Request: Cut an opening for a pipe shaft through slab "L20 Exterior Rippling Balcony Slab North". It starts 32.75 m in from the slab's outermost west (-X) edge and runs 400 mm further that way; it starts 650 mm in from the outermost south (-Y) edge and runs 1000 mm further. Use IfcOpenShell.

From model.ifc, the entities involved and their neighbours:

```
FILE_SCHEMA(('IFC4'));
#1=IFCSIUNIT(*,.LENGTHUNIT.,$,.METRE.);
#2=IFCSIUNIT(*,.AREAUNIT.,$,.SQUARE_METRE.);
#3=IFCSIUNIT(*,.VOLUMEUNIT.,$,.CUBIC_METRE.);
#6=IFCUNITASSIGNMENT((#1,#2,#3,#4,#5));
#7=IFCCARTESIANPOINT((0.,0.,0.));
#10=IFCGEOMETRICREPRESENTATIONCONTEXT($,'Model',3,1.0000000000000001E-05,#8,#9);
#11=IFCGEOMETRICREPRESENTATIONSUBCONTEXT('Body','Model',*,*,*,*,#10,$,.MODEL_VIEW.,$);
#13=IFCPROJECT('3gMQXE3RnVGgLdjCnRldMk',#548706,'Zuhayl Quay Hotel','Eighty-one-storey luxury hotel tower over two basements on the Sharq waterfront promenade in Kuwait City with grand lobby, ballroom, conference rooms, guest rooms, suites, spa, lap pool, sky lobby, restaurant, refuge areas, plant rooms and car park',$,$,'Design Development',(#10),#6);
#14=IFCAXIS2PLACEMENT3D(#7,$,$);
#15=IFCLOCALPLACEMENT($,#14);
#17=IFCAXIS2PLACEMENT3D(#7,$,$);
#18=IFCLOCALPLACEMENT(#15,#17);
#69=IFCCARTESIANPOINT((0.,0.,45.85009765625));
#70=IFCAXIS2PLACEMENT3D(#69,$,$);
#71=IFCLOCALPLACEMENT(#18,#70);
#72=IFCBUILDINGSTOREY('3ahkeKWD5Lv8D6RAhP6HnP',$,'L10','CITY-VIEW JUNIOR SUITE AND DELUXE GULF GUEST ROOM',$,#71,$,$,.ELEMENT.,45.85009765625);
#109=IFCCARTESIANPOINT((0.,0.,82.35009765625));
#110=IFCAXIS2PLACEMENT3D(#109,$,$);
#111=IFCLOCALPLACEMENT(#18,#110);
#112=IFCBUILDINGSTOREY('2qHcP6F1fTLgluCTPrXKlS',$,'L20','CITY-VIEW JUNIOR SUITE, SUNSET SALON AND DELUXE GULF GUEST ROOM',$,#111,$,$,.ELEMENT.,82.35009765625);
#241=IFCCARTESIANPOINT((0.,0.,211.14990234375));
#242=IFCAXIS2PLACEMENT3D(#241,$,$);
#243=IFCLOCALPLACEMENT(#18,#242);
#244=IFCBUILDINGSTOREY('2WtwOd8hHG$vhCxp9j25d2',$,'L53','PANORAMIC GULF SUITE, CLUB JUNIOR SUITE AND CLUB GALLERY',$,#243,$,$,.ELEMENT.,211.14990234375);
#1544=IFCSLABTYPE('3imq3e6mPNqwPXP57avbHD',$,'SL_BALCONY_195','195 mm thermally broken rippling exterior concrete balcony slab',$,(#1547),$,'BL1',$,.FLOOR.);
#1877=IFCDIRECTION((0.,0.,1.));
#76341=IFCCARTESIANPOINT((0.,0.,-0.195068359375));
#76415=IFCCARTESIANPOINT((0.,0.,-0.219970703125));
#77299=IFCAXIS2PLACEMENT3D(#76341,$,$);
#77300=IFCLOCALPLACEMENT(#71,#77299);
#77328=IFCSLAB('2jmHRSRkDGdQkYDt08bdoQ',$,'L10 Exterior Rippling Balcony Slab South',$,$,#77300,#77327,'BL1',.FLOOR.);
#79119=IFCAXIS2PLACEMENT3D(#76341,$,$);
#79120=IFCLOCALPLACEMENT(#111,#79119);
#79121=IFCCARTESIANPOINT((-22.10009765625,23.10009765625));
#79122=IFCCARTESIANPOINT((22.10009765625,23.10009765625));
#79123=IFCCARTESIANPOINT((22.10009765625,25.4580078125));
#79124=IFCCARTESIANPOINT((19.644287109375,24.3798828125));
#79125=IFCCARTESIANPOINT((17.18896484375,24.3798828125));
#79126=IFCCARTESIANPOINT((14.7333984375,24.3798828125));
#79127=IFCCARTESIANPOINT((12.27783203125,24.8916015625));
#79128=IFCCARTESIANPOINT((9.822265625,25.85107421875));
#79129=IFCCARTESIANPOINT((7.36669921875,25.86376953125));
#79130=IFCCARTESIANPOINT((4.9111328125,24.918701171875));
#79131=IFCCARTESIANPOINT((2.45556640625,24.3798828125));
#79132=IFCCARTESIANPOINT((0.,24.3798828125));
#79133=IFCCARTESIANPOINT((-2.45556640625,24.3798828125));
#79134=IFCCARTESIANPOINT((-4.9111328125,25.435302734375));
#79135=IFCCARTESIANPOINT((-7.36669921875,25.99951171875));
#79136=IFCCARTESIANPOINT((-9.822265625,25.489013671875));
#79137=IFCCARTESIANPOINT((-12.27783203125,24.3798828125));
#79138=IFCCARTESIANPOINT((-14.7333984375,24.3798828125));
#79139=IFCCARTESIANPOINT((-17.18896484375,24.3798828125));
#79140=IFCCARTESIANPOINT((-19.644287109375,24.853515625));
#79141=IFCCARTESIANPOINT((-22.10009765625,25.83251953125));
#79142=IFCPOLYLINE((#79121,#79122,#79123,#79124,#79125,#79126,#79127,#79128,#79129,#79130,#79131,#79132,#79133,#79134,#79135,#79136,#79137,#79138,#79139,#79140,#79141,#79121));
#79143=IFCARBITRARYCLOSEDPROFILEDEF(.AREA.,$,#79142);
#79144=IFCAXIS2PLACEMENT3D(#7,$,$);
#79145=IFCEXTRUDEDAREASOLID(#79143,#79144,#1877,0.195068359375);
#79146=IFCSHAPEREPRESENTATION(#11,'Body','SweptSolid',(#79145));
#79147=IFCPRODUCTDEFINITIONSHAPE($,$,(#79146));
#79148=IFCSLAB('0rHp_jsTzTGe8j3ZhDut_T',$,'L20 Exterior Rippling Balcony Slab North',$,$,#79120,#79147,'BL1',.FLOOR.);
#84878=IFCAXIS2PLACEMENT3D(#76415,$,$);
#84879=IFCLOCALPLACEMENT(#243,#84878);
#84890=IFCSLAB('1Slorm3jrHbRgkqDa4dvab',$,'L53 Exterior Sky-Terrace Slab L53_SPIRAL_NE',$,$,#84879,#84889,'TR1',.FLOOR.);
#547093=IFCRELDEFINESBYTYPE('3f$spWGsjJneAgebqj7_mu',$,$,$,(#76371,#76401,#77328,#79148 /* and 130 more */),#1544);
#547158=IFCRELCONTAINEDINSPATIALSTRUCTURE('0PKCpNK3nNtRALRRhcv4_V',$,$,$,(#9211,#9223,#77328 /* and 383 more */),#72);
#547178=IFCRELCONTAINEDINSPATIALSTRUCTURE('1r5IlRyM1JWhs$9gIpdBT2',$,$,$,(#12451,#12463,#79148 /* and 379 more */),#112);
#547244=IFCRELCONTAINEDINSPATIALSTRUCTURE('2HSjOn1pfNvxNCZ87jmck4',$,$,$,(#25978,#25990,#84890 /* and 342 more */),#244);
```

```python
import numpy as np
import ifcopenshell
import ifcopenshell.api.feature
import ifcopenshell.api.geometry
import ifcopenshell.api.root
import ifcopenshell.geom
import ifcopenshell.util.placement
import ifcopenshell.util.representation
import ifcopenshell.util.shape
import ifcopenshell.util.unit

model = ifcopenshell.open("model.ifc")
unit_scale = ifcopenshell.util.unit.calculate_unit_scale(model)
settings = ifcopenshell.geom.settings()


def volume(element):
    """Net volume in cubic metres, openings subtracted."""
    shape = ifcopenshell.geom.create_shape(settings, element)
    return ifcopenshell.util.shape.get_volume(shape.geometry)


slab = model.by_guid("0rHp_jsTzTGe8j3ZhDut_T")
before = volume(slab)

# Extent in the slab's own axes, in metres. The edges named are its -X and -Y sides.
slab_shape = ifcopenshell.geom.create_shape(settings, slab)
vertices = ifcopenshell.util.shape.get_vertices(slab_shape.geometry)
x_min, y_min, bottom = vertices.min(axis=0)
top = vertices[:, 2].max()

opening = ifcopenshell.api.root.create_entity(model, ifc_class="IfcOpeningElement", name="Pipe shaft opening", predefined_type="OPENING")
context = ifcopenshell.util.representation.get_context(model, "Model", "Body", "MODEL_VIEW")
width, depth = 0.4, 1
outline = [(0.0, 0.0), (width, 0.0), (width, depth), (0.0, depth), (0.0, 0.0)]
# Overshoot both faces by 50 mm so the cut is clean.
shape = ifcopenshell.api.geometry.add_slab_representation(
    model, context=context, depth=top - bottom + 0.1, polyline=outline
)
ifcopenshell.api.geometry.assign_representation(model, product=opening, representation=shape)

matrix = ifcopenshell.util.placement.get_local_placement(slab.ObjectPlacement)
matrix[:, 3] = matrix @ np.append(np.array([x_min + 32.75, y_min + 0.65, bottom - 0.05]) / unit_scale, 1.0)
ifcopenshell.api.geometry.edit_object_placement(model, product=opening, matrix=matrix, is_si=False)
ifcopenshell.api.feature.add_feature(model, feature=opening, element=slab)

after = volume(slab)

print(f"slab volume {before:.3f} -> {after:.3f} m3")

model.write("model_updated.ifc")
```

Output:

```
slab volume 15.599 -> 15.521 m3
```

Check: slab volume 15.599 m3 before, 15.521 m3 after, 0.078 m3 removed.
